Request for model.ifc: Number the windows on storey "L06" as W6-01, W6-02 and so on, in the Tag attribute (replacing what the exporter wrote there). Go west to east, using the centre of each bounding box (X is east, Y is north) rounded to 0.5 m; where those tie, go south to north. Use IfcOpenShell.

First a look at what the model holds.

```python
import ifcopenshell
import ifcopenshell.util.element
import ifcopenshell.util.placement

model = ifcopenshell.open("model.ifc")
print(model.schema)
storey = next(s for s in model.by_type("IfcBuildingStorey") if s.Name == "L06")
windows = [e for e in ifcopenshell.util.element.get_decomposition(storey) if e.is_a("IfcWindow")]
for e in sorted(windows, key=lambda e: e.id()):
    origin = ifcopenshell.util.placement.get_local_placement(e.ObjectPlacement)[:3, 3]
    print(e.id(), e.Tag, e.Name, origin.round(2) + 0.0, sep=" | ")
```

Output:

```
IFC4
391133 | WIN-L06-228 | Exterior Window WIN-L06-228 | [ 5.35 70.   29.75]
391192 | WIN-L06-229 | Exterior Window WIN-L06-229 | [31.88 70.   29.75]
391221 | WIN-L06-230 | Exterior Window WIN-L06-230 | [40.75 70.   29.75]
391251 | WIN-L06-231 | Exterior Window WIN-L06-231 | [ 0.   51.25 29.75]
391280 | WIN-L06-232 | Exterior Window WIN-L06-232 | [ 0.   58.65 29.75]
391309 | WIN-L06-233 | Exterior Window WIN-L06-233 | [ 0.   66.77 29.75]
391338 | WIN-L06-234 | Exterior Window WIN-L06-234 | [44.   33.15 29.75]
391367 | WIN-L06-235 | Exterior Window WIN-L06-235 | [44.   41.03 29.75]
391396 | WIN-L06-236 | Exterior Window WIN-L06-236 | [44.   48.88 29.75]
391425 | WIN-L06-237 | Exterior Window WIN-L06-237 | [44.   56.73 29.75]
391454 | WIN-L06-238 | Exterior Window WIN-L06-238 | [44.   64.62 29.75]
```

```python
import ifcopenshell
import ifcopenshell.geom
import ifcopenshell.util.element
import ifcopenshell.util.shape

model = ifcopenshell.open("model.ifc")
settings = ifcopenshell.geom.settings()
settings.set("use-world-coords", True)


def centre(element):
    shape = ifcopenshell.geom.create_shape(settings, element)
    return ifcopenshell.util.shape.get_bbox_centroid(shape.geometry)


storey = next(s for s in model.by_type("IfcBuildingStorey") if s.Name == "L06")
windows = [e for e in ifcopenshell.util.element.get_decomposition(storey) if e.is_a("IfcWindow")]

# Insertion points can sit at a corner or the storey origin, so sort by the geometry (in metres).
centres = {e: centre(e) for e in windows}
windows.sort(key=lambda e: (round(centres[e][0] / 0.5), centres[e][1]))

for i, e in enumerate(windows, start=1):
    number = f"W6-{i:02d}"
    e.Tag = number
    print(e.id(), number)

model.write("model-out.ifc")
```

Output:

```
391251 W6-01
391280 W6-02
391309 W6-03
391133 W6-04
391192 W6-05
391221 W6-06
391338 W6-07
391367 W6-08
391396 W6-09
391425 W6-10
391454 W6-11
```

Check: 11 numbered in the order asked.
